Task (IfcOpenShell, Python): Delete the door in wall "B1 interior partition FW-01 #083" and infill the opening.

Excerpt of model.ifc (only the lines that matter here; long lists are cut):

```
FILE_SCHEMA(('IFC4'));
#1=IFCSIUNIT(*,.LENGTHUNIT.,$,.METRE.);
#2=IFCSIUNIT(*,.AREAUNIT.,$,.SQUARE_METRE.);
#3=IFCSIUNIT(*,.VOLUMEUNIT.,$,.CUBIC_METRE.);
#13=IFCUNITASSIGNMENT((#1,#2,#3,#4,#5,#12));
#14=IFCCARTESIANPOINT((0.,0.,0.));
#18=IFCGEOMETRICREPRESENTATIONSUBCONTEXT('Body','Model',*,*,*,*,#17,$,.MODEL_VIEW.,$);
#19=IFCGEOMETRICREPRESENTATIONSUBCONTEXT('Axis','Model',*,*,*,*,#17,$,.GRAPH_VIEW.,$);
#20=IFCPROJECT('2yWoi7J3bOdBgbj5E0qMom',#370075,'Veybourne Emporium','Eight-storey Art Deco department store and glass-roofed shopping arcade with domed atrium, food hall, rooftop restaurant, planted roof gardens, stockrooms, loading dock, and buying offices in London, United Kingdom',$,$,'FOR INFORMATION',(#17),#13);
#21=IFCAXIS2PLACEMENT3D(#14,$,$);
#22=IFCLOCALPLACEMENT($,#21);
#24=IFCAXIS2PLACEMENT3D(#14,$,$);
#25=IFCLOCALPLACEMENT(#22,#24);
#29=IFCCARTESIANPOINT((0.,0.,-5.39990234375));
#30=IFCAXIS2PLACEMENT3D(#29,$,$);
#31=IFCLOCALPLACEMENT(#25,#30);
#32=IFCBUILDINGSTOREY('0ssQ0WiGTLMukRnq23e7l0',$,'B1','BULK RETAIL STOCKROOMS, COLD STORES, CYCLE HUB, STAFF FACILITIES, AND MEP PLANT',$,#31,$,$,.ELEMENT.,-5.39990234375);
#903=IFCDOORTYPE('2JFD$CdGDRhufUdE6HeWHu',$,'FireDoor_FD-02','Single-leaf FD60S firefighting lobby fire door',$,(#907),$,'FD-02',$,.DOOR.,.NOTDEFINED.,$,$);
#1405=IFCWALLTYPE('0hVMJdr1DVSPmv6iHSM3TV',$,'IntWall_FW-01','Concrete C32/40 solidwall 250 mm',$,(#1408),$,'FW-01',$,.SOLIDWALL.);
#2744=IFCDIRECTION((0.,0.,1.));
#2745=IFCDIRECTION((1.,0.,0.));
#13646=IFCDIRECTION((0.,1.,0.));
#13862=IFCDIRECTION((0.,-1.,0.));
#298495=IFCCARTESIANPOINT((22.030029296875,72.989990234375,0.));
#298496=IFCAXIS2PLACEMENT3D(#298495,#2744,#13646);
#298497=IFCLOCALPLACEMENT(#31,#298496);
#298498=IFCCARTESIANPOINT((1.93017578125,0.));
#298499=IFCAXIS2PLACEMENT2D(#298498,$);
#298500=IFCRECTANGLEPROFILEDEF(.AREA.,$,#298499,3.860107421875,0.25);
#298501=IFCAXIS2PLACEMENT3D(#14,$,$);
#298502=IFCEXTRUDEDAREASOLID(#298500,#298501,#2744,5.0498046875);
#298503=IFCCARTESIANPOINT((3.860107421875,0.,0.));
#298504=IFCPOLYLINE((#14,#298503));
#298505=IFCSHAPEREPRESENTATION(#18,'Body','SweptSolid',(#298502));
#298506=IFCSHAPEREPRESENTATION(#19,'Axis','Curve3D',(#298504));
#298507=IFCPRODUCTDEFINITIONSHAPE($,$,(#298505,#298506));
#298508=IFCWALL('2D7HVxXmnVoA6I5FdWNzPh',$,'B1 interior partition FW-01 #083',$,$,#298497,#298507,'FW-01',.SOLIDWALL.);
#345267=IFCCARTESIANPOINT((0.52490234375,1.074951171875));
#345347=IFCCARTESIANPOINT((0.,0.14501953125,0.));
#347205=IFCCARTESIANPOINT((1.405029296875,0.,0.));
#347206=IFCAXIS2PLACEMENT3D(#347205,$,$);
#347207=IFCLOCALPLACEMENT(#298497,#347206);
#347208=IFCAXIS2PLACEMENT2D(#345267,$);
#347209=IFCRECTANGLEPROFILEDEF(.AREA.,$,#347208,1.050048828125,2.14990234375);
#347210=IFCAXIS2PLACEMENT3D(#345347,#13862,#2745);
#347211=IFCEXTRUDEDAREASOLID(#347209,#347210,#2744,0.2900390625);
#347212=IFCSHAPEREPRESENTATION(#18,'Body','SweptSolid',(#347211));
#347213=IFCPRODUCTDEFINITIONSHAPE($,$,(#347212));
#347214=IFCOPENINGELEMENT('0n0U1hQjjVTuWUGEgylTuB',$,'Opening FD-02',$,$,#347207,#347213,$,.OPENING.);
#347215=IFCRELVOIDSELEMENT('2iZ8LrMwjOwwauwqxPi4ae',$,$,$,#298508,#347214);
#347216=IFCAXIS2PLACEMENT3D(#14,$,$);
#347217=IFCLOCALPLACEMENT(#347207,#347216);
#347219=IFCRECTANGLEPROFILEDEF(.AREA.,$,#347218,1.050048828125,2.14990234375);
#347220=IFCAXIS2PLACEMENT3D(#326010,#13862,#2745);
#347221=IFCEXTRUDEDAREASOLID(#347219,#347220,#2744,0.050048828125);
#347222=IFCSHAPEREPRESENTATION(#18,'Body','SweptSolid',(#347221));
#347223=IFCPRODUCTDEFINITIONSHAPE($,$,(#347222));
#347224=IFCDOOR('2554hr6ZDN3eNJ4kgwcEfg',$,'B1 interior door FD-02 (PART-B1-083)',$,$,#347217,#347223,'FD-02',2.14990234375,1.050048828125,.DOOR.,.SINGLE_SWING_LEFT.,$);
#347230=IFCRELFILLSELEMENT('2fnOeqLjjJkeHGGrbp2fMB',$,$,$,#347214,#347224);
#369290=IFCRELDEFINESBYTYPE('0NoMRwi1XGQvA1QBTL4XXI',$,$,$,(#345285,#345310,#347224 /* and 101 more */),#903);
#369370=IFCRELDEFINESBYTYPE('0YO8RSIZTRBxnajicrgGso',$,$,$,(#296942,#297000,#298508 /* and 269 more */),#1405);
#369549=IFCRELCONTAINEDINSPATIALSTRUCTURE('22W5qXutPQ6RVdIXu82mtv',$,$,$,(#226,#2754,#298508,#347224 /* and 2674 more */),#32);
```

```python
import ifcopenshell
import ifcopenshell.api.feature
import ifcopenshell.api.root
import ifcopenshell.geom
import ifcopenshell.util.shape

model = ifcopenshell.open("model.ifc")
settings = ifcopenshell.geom.settings()


def volume(element):
    """Net volume in cubic metres, openings subtracted."""
    shape = ifcopenshell.geom.create_shape(settings, element)
    return ifcopenshell.util.shape.get_volume(shape.geometry)


door = model.by_guid("2554hr6ZDN3eNJ4kgwcEfg")
opening = door.FillsVoids[0].RelatingOpeningElement
wall = opening.VoidsElements[0].RelatingBuildingElement
before = volume(wall)

ifcopenshell.api.root.remove_product(model, product=door)
ifcopenshell.api.feature.remove_feature(model, feature=opening)

after = volume(wall)

print(f"wall volume {before:.3f} -> {after:.3f} m3")

model.write("model_v2.ifc")
```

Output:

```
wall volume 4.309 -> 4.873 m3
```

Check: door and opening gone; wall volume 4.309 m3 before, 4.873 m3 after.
